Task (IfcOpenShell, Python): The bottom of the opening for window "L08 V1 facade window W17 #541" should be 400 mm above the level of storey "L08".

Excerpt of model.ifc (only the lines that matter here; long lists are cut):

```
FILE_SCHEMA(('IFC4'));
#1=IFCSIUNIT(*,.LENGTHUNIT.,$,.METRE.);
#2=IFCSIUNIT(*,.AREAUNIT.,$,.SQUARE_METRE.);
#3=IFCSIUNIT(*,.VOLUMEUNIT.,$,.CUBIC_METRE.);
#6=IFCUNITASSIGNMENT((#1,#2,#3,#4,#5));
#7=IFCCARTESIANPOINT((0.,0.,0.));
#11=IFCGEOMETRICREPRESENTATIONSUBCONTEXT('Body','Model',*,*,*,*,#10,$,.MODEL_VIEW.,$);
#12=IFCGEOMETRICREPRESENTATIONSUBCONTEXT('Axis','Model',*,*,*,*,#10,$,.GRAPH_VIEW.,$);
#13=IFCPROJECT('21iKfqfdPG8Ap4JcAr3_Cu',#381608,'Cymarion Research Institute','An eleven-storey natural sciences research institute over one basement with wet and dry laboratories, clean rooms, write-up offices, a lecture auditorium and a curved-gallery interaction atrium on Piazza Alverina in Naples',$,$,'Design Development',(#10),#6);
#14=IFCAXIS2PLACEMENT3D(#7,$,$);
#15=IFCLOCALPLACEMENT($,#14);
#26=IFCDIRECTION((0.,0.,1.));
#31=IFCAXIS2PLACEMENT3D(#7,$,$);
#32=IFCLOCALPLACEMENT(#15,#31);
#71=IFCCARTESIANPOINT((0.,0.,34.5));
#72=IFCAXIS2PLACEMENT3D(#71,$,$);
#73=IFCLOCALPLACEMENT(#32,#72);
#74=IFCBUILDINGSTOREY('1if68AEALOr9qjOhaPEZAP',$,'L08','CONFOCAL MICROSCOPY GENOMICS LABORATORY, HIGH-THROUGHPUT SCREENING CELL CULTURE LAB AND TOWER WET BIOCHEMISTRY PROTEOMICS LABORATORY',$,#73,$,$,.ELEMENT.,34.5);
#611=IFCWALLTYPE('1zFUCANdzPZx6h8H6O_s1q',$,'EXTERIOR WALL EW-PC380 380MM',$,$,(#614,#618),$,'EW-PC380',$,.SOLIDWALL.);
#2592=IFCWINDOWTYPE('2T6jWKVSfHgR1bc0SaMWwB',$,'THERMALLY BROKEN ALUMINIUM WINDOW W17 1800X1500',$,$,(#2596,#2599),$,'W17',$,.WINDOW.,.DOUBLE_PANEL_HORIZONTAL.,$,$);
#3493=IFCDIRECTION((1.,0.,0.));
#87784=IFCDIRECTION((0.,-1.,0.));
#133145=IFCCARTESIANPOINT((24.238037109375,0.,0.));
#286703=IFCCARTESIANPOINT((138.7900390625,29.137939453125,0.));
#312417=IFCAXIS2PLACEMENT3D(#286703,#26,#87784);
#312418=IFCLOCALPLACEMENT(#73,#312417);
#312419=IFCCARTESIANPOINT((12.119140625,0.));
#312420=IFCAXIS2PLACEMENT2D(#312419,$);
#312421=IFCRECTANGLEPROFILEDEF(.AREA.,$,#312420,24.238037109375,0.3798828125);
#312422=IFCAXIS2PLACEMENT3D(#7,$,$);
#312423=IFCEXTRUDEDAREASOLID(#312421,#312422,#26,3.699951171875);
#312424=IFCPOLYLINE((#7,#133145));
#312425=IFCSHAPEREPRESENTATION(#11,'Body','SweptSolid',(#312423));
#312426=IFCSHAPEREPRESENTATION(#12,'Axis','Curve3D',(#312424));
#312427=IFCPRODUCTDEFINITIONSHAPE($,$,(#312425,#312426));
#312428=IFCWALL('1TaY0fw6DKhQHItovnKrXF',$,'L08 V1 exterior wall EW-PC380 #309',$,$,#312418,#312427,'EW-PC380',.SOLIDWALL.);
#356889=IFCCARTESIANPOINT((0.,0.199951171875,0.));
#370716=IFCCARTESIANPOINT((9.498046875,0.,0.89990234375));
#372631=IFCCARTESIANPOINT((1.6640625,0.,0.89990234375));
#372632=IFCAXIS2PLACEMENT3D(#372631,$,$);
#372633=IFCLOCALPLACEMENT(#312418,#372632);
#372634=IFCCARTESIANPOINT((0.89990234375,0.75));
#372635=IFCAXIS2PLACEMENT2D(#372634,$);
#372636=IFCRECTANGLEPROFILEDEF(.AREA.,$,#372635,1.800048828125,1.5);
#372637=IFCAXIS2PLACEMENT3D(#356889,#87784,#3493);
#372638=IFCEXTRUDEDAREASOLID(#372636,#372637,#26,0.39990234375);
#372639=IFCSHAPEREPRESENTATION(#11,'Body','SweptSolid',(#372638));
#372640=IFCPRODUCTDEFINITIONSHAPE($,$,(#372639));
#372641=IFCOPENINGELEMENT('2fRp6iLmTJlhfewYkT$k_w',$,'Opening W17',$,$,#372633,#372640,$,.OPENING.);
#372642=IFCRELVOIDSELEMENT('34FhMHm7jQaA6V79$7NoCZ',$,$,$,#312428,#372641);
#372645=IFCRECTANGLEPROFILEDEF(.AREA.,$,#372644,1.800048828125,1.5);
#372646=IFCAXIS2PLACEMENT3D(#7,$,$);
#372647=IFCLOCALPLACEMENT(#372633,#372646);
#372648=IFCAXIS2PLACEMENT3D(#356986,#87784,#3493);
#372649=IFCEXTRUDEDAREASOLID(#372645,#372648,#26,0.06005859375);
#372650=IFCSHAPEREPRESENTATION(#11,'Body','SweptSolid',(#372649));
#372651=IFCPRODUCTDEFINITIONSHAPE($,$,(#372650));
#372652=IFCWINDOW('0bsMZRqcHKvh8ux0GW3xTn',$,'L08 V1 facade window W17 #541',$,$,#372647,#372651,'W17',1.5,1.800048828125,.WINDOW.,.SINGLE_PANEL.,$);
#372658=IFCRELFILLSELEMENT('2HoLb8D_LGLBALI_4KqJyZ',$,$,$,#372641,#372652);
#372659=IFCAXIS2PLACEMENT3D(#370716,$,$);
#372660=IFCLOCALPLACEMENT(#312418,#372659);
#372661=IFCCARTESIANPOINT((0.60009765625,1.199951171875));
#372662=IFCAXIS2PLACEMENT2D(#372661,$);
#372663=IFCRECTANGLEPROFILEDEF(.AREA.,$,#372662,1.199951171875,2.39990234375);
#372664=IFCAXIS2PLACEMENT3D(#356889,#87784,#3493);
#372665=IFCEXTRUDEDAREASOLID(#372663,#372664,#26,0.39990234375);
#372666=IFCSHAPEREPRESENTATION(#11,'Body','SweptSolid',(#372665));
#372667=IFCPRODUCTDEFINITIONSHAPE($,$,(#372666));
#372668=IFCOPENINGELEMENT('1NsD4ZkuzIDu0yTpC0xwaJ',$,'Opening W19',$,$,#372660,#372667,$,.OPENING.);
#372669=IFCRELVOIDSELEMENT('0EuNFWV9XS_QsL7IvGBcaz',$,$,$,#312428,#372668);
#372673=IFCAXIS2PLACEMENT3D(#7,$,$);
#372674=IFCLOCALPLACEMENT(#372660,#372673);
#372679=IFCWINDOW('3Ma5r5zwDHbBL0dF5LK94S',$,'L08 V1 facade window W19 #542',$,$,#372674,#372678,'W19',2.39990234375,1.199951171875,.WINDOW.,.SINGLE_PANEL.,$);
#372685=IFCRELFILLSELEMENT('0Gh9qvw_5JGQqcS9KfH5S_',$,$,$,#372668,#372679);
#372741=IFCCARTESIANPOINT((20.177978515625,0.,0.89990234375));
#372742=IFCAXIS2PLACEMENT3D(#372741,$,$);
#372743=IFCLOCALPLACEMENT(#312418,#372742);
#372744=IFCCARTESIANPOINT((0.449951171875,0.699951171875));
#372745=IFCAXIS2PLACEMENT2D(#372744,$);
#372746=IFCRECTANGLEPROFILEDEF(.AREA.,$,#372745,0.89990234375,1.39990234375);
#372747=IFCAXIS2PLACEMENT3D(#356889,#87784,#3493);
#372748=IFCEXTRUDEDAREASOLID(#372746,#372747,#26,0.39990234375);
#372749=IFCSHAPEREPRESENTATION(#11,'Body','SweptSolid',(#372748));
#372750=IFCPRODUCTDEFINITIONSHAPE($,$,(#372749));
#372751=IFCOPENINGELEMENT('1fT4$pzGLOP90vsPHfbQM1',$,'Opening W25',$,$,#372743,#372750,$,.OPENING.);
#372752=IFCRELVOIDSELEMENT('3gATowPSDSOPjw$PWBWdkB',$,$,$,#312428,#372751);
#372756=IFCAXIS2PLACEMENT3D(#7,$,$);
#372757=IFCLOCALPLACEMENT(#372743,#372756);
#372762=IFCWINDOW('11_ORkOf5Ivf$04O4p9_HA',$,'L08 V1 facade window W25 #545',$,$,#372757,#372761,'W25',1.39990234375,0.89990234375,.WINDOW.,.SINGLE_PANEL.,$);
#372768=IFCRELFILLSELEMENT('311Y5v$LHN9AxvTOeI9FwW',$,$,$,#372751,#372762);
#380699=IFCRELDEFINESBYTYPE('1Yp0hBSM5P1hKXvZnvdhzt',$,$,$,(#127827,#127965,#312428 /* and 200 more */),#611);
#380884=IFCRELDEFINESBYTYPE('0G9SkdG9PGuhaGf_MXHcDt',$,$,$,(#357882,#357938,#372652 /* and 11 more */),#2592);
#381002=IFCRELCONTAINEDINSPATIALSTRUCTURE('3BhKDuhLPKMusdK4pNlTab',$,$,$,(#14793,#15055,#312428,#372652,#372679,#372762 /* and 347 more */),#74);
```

```python
import numpy as np
import ifcopenshell
import ifcopenshell.api.geometry
import ifcopenshell.geom
import ifcopenshell.util.element
import ifcopenshell.util.placement
import ifcopenshell.util.shape
import ifcopenshell.util.unit

model = ifcopenshell.open("model.ifc")
unit_scale = ifcopenshell.util.unit.calculate_unit_scale(model)

window = model.by_guid("0bsMZRqcHKvh8ux0GW3xTn")
opening = window.FillsVoids[0].RelatingOpeningElement
storey = ifcopenshell.util.element.get_container(window, ifc_class="IfcBuildingStorey")
level = ifcopenshell.util.placement.get_local_placement(storey.ObjectPlacement)[2, 3]

# The opening's origin need not be at the sill, so measure its lowest point.
shape = ifcopenshell.geom.create_shape(ifcopenshell.geom.settings(), opening)
bottom = ifcopenshell.util.shape.get_shape_bottom_elevation(shape, shape.geometry) / unit_scale
dz = level + 0.4 / unit_scale - bottom

shift = np.array([0.0, 0.0, dz])
# The window is placed relative to its opening, so it follows when the opening moves.
matrix = ifcopenshell.util.placement.get_local_placement(opening.ObjectPlacement)
matrix[:3, 3] += shift
ifcopenshell.api.geometry.edit_object_placement(
    model, product=opening, matrix=matrix, is_si=False, should_transform_children=True
)

print(f"moved by {dz * unit_scale:+.3f} m")

model.write("model_v2.ifc")
```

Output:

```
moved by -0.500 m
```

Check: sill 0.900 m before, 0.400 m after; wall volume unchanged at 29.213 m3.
